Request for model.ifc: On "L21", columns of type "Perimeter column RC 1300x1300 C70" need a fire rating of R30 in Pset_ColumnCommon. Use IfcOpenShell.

First a look at what the model holds.

```python
import ifcopenshell
import ifcopenshell.util.element

model = ifcopenshell.open("model.ifc")
print(model.schema)
storey = next(s for s in model.by_type("IfcBuildingStorey") if s.Name == "L21")
columns = [e for e in ifcopenshell.util.element.get_decomposition(storey) if e.is_a("IfcColumn")]
seen = {}
for e in columns:
    element_type = ifcopenshell.util.element.get_type(e)
    key = (element_type.Name if element_type != e and element_type else None, ifcopenshell.util.element.get_pset(e, "Pset_ColumnCommon", "FireRating"))
    seen[key] = seen.get(key, 0) + 1
for (name, value), count in sorted(seen.items(), key=str):
    print(count, "x", name, "|", value)
```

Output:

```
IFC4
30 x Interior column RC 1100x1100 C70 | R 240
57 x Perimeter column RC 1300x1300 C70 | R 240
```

```python
import ifcopenshell
import ifcopenshell.api.pset
import ifcopenshell.util.element

model = ifcopenshell.open("model.ifc")

storey = next(s for s in model.by_type("IfcBuildingStorey") if s.Name == "L21")
columns = [e for e in ifcopenshell.util.element.get_decomposition(storey) if e.is_a("IfcColumn")]

count = 0
for e in columns:
    element_type = ifcopenshell.util.element.get_type(e)
    if element_type in (None, e) or element_type.Name != "Perimeter column RC 1300x1300 C70":
        continue
    found = ifcopenshell.util.element.get_pset(e, "Pset_ColumnCommon", should_inherit=False)
    if found:
        pset = model.by_id(found["id"])
        if len(ifcopenshell.util.element.get_elements_by_pset(pset)) > 1:
            pset = ifcopenshell.api.pset.unshare_pset(model, products=[e], pset=pset)[0]
    else:
        pset = ifcopenshell.api.pset.add_pset(model, product=e, name="Pset_ColumnCommon")
    ifcopenshell.api.pset.edit_pset(model, pset=pset, properties={"FireRating": "R30"})
    count += 1

print(count, "columns updated")

model.write("model_rev.ifc")
```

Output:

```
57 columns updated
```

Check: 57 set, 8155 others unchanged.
